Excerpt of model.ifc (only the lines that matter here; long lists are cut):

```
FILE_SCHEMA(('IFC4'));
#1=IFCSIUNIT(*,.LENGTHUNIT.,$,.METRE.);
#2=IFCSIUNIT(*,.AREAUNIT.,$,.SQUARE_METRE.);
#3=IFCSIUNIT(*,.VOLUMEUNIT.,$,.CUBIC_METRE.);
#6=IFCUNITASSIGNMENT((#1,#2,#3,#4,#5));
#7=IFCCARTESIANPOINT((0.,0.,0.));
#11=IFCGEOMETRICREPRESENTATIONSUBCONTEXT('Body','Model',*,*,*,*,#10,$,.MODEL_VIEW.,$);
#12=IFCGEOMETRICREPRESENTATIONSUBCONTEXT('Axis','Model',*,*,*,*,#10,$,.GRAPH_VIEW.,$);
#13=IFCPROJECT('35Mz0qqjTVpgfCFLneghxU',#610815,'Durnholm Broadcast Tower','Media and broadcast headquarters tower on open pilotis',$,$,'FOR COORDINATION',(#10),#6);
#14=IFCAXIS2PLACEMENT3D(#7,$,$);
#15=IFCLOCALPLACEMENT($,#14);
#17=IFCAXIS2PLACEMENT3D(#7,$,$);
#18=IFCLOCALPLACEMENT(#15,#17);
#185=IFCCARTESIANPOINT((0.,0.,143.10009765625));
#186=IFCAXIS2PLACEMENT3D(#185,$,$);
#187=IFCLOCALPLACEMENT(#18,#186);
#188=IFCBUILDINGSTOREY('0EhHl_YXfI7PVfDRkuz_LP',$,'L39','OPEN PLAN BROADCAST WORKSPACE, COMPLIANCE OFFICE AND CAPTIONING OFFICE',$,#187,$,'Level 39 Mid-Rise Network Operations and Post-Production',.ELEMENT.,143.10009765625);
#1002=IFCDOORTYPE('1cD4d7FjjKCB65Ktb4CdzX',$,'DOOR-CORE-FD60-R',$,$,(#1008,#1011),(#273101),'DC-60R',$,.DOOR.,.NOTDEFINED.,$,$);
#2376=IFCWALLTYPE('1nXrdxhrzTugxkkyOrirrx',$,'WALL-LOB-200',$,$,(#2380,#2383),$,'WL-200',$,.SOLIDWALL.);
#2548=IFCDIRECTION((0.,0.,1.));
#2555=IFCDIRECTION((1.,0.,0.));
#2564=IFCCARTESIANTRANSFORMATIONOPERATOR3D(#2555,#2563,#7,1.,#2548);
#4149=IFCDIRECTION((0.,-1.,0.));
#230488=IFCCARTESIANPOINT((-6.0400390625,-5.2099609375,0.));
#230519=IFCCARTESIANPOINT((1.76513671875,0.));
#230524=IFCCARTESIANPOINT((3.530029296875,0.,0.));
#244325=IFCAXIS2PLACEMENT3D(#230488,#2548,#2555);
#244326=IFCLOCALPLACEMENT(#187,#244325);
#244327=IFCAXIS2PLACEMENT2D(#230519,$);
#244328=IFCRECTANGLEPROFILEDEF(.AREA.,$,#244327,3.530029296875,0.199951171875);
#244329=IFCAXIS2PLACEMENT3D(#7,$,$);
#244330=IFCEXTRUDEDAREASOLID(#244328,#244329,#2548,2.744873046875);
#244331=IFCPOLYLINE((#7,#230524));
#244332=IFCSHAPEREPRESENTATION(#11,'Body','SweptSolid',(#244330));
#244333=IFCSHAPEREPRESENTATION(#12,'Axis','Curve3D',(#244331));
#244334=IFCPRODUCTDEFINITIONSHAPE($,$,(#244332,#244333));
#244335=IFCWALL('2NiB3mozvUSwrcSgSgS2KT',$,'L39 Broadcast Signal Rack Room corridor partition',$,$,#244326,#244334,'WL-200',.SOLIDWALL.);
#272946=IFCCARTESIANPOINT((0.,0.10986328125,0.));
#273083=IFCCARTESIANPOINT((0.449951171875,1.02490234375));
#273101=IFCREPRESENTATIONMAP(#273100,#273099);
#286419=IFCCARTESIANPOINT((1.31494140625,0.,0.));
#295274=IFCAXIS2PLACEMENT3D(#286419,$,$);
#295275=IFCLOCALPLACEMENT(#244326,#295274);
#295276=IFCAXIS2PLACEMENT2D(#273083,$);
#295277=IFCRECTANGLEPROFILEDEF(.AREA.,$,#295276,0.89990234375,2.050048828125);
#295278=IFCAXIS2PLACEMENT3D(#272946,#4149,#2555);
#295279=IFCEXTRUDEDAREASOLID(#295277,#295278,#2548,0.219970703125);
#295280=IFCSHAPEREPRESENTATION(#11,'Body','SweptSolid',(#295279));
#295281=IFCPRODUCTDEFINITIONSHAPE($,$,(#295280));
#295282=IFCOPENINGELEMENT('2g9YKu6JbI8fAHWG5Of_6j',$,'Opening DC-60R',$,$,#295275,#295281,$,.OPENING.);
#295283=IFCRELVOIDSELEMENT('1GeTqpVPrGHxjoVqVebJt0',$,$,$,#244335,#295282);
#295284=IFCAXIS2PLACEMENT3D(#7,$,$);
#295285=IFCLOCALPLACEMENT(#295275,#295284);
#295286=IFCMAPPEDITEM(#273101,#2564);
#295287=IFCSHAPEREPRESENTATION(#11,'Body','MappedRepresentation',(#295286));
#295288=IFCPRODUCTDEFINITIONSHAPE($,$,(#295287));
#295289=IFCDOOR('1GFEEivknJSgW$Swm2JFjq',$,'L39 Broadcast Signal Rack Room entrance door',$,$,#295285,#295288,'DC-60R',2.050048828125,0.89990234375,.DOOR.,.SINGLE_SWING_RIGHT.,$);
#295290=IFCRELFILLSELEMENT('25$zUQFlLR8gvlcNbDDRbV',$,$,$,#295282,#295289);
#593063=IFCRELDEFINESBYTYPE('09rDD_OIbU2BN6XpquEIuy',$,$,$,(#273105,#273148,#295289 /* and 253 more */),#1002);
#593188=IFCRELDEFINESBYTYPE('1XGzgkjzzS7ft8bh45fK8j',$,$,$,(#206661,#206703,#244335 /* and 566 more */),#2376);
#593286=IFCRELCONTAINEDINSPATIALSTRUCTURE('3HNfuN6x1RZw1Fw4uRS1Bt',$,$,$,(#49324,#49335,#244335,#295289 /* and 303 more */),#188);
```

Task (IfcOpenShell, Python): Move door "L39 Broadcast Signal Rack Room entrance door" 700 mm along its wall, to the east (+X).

```python
import ifcopenshell
import ifcopenshell.api.geometry
import ifcopenshell.util.placement
import ifcopenshell.util.unit

model = ifcopenshell.open("model.ifc")
unit_scale = ifcopenshell.util.unit.calculate_unit_scale(model)

door = model.by_guid("1GFEEivknJSgW$Swm2JFjq")
opening = door.FillsVoids[0].RelatingOpeningElement
wall = opening.VoidsElements[0].RelatingBuildingElement

wall_matrix = ifcopenshell.util.placement.get_local_placement(wall.ObjectPlacement)
shift = wall_matrix[:3, 0] * 0.7 / unit_scale
before = ifcopenshell.util.placement.get_local_placement(door.ObjectPlacement)[:3, 3].copy()

# The door is placed relative to its opening, so it follows when the opening moves.
matrix = ifcopenshell.util.placement.get_local_placement(opening.ObjectPlacement)
matrix[:3, 3] += shift
ifcopenshell.api.geometry.edit_object_placement(
    model, product=opening, matrix=matrix, is_si=False, should_transform_children=True
)

after = ifcopenshell.util.placement.get_local_placement(door.ObjectPlacement)[:3, 3]
print("door moved by", (after - before).round(3) + 0.0)

model.write("model_edited.ifc")
```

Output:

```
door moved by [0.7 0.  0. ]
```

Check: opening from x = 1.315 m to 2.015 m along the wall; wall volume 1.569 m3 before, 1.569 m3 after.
